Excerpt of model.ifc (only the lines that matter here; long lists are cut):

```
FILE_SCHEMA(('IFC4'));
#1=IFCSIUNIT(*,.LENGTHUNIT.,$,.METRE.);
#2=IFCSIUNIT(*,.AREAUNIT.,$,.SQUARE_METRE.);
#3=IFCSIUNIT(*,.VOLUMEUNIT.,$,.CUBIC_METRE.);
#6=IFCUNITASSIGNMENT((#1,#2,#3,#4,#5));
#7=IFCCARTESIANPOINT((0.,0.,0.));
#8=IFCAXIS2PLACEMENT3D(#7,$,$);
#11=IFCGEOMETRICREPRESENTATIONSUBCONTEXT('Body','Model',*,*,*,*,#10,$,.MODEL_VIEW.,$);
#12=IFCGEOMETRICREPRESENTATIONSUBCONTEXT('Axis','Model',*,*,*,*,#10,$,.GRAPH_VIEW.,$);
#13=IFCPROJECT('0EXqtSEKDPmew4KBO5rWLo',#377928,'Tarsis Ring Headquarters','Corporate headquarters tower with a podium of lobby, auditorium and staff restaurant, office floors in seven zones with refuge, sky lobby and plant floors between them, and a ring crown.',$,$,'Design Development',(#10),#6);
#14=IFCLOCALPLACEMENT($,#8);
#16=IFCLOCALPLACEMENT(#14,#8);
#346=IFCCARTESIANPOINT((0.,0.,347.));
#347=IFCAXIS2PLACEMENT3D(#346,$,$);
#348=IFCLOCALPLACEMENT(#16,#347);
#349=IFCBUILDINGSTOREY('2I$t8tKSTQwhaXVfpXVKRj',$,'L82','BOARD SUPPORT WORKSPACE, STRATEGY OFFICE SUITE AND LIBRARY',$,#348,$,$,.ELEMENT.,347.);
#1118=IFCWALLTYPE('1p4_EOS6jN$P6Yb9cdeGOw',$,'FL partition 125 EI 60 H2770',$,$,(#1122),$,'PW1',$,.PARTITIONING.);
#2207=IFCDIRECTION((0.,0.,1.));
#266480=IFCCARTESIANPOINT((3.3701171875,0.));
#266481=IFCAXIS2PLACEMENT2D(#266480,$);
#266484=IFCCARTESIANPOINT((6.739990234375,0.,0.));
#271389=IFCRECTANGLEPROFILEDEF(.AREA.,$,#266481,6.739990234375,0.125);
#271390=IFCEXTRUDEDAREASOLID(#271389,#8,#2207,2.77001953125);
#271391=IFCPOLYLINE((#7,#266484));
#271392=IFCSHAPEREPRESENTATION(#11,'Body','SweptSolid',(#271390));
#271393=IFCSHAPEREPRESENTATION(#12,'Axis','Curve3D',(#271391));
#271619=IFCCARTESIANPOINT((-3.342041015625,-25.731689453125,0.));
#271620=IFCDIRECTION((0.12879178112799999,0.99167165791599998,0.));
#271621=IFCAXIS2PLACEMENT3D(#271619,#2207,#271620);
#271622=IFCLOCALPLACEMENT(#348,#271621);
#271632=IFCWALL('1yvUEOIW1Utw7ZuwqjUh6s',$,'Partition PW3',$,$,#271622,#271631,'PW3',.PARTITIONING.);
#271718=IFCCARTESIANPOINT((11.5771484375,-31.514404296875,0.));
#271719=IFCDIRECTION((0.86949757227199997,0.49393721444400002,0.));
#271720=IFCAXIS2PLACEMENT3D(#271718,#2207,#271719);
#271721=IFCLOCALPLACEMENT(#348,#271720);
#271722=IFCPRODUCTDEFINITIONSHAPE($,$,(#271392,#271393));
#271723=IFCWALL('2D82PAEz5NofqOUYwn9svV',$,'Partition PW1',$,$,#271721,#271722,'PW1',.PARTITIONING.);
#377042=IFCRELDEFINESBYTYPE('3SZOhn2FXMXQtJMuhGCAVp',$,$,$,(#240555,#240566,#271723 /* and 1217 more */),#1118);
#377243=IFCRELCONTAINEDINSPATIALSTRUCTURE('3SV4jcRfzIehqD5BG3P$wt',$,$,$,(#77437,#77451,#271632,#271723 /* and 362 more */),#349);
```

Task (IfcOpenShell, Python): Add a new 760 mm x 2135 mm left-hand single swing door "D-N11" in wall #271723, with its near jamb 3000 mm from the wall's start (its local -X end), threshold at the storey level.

```python
import numpy as np
import ifcopenshell
import ifcopenshell.api.feature
import ifcopenshell.api.geometry
import ifcopenshell.api.root
import ifcopenshell.api.spatial
import ifcopenshell.geom
import ifcopenshell.util.element
import ifcopenshell.util.placement
import ifcopenshell.util.representation
import ifcopenshell.util.shape
import ifcopenshell.util.unit

model = ifcopenshell.open("model.ifc")
unit_scale = ifcopenshell.util.unit.calculate_unit_scale(model)
settings = ifcopenshell.geom.settings()


def volume(element):
    """Net volume in cubic metres, openings subtracted."""
    shape = ifcopenshell.geom.create_shape(settings, element)
    return ifcopenshell.util.shape.get_volume(shape.geometry)


wall = model.by_guid("2D82PAEz5NofqOUYwn9svV")
storey = ifcopenshell.util.element.get_container(wall, ifc_class="IfcBuildingStorey")
context = ifcopenshell.util.representation.get_context(model, "Model", "Body", "MODEL_VIEW")
before = volume(wall)

width, height, from_end, sill = 0.76, 2.135, 3, 0.0  # metres

# The wall runs along its own X axis, and the end named is its -X end.
wall_shape = ifcopenshell.geom.create_shape(settings, wall)
x, y, z = ifcopenshell.util.shape.get_vertices(wall_shape.geometry).T
start = x.min() + from_end
face, thickness = float(y.min()), float(y.max() - y.min())
wall_matrix = ifcopenshell.util.placement.get_local_placement(wall.ObjectPlacement)
level = ifcopenshell.util.placement.get_local_placement(storey.ObjectPlacement)[2, 3]


def in_wall(x, y):
    """Placement at x, y metres in the wall's axes, at sill height."""
    matrix = wall_matrix.copy()
    matrix[:, 3] = wall_matrix @ np.array([x / unit_scale, y / unit_scale, 0.0, 1.0])
    matrix[2, 3] = level + sill / unit_scale
    return matrix


# Opening: a box that overshoots both wall faces by 50 mm.
opening = ifcopenshell.api.root.create_entity(model, ifc_class="IfcOpeningElement", predefined_type="OPENING")
box = ifcopenshell.api.geometry.add_wall_representation(
    model, context=context, length=width, height=height, thickness=thickness + 0.1
)
ifcopenshell.api.geometry.assign_representation(model, product=opening, representation=box)
ifcopenshell.api.geometry.edit_object_placement(model, product=opening, matrix=in_wall(start, face - 0.05), is_si=False)
ifcopenshell.api.feature.add_feature(model, feature=opening, element=wall)

door = ifcopenshell.api.root.create_entity(model, ifc_class="IfcDoor", name="D-N11", predefined_type="DOOR")
door.OverallWidth, door.OverallHeight = width / unit_scale, height / unit_scale
door.OperationType = "SINGLE_SWING_LEFT"
body = ifcopenshell.api.geometry.add_door_representation(
    model,
    context=context,
    overall_width=door.OverallWidth,
    overall_height=door.OverallHeight,
    operation_type="SINGLE_SWING_LEFT",
    lining_properties={"LiningDepth": thickness / unit_scale, "ThresholdDepth": thickness / unit_scale},
)
ifcopenshell.api.geometry.assign_representation(model, product=door, representation=body)
ifcopenshell.api.spatial.assign_container(model, products=[door], relating_structure=storey)
ifcopenshell.api.feature.add_filling(model, opening=opening, element=door)

# The lining spans the wall, so the door starts at the wall face.
ifcopenshell.api.geometry.edit_object_placement(model, product=door, matrix=in_wall(start, face), is_si=False)

after = volume(wall)

print(f"wall volume {before:.3f} -> {after:.3f} m3")

model.write("model_rev.ifc")
```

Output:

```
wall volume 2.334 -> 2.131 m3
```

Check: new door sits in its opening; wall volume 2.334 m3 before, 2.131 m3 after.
